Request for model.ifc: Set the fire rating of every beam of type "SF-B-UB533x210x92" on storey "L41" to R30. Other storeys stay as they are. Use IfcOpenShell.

First a look at what the model holds.

```python
import ifcopenshell
import ifcopenshell.util.element

model = ifcopenshell.open("model.ifc")
print(model.schema)
storey = next(s for s in model.by_type("IfcBuildingStorey") if s.Name == "L41")
beams = [e for e in ifcopenshell.util.element.get_decomposition(storey) if e.is_a("IfcBeam")]
seen = {}
for e in beams:
    element_type = ifcopenshell.util.element.get_type(e)
    key = (element_type.Name if element_type != e and element_type else None, ifcopenshell.util.element.get_pset(e, "Pset_BeamCommon", "FireRating"))
    seen[key] = seen.get(key, 0) + 1
for (name, value), count in sorted(seen.items(), key=str):
    print(count, "x", name, "|", value)
```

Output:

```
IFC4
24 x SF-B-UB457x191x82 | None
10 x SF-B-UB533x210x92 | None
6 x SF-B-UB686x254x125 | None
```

```python
import ifcopenshell
import ifcopenshell.api.pset
import ifcopenshell.util.element

model = ifcopenshell.open("model.ifc")

storey = next(s for s in model.by_type("IfcBuildingStorey") if s.Name == "L41")
beams = [e for e in ifcopenshell.util.element.get_decomposition(storey) if e.is_a("IfcBeam")]

count = 0
for e in beams:
    element_type = ifcopenshell.util.element.get_type(e)
    if element_type in (None, e) or element_type.Name != "SF-B-UB533x210x92":
        continue
    found = ifcopenshell.util.element.get_pset(e, "Pset_BeamCommon", should_inherit=False)
    if found:
        pset = model.by_id(found["id"])
        if len(ifcopenshell.util.element.get_elements_by_pset(pset)) > 1:
            pset = ifcopenshell.api.pset.unshare_pset(model, products=[e], pset=pset)[0]
    else:
        pset = ifcopenshell.api.pset.add_pset(model, product=e, name="Pset_BeamCommon")
    ifcopenshell.api.pset.edit_pset(model, pset=pset, properties={"FireRating": "R30"})
    count += 1

print(count, "beams updated")

model.write("model_edited.ifc")
```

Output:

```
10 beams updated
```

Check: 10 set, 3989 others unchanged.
